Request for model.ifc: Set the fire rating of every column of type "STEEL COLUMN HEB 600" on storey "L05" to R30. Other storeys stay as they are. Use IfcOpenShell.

First a look at what the model holds.

```python
import ifcopenshell
import ifcopenshell.util.element

model = ifcopenshell.open("model.ifc")
print(model.schema)
storey = next(s for s in model.by_type("IfcBuildingStorey") if s.Name == "L05")
columns = [e for e in ifcopenshell.util.element.get_decomposition(storey) if e.is_a("IfcColumn")]
seen = {}
for e in columns:
    element_type = ifcopenshell.util.element.get_type(e)
    key = (element_type.Name if element_type != e and element_type else None, ifcopenshell.util.element.get_pset(e, "Pset_ColumnCommon", "FireRating"))
    seen[key] = seen.get(key, 0) + 1
for (name, value), count in sorted(seen.items(), key=str):
    print(count, "x", name, "|", value)
```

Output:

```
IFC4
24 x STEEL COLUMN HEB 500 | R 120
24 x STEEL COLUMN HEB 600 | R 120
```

```python
import ifcopenshell
import ifcopenshell.api.pset
import ifcopenshell.util.element

model = ifcopenshell.open("model.ifc")

storey = next(s for s in model.by_type("IfcBuildingStorey") if s.Name == "L05")
columns = [e for e in ifcopenshell.util.element.get_decomposition(storey) if e.is_a("IfcColumn")]

count = 0
for e in columns:
    element_type = ifcopenshell.util.element.get_type(e)
    if element_type in (None, e) or element_type.Name != "STEEL COLUMN HEB 600":
        continue
    # add_pset returns the element's existing set when there is one.
    pset = ifcopenshell.api.pset.add_pset(model, product=e, name="Pset_ColumnCommon")
    ifcopenshell.api.pset.edit_pset(model, pset=pset, properties={"FireRating": "R30"})
    count += 1

print(count, "columns updated")

model.write("model_edited.ifc")
```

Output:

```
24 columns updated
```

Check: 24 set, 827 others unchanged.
